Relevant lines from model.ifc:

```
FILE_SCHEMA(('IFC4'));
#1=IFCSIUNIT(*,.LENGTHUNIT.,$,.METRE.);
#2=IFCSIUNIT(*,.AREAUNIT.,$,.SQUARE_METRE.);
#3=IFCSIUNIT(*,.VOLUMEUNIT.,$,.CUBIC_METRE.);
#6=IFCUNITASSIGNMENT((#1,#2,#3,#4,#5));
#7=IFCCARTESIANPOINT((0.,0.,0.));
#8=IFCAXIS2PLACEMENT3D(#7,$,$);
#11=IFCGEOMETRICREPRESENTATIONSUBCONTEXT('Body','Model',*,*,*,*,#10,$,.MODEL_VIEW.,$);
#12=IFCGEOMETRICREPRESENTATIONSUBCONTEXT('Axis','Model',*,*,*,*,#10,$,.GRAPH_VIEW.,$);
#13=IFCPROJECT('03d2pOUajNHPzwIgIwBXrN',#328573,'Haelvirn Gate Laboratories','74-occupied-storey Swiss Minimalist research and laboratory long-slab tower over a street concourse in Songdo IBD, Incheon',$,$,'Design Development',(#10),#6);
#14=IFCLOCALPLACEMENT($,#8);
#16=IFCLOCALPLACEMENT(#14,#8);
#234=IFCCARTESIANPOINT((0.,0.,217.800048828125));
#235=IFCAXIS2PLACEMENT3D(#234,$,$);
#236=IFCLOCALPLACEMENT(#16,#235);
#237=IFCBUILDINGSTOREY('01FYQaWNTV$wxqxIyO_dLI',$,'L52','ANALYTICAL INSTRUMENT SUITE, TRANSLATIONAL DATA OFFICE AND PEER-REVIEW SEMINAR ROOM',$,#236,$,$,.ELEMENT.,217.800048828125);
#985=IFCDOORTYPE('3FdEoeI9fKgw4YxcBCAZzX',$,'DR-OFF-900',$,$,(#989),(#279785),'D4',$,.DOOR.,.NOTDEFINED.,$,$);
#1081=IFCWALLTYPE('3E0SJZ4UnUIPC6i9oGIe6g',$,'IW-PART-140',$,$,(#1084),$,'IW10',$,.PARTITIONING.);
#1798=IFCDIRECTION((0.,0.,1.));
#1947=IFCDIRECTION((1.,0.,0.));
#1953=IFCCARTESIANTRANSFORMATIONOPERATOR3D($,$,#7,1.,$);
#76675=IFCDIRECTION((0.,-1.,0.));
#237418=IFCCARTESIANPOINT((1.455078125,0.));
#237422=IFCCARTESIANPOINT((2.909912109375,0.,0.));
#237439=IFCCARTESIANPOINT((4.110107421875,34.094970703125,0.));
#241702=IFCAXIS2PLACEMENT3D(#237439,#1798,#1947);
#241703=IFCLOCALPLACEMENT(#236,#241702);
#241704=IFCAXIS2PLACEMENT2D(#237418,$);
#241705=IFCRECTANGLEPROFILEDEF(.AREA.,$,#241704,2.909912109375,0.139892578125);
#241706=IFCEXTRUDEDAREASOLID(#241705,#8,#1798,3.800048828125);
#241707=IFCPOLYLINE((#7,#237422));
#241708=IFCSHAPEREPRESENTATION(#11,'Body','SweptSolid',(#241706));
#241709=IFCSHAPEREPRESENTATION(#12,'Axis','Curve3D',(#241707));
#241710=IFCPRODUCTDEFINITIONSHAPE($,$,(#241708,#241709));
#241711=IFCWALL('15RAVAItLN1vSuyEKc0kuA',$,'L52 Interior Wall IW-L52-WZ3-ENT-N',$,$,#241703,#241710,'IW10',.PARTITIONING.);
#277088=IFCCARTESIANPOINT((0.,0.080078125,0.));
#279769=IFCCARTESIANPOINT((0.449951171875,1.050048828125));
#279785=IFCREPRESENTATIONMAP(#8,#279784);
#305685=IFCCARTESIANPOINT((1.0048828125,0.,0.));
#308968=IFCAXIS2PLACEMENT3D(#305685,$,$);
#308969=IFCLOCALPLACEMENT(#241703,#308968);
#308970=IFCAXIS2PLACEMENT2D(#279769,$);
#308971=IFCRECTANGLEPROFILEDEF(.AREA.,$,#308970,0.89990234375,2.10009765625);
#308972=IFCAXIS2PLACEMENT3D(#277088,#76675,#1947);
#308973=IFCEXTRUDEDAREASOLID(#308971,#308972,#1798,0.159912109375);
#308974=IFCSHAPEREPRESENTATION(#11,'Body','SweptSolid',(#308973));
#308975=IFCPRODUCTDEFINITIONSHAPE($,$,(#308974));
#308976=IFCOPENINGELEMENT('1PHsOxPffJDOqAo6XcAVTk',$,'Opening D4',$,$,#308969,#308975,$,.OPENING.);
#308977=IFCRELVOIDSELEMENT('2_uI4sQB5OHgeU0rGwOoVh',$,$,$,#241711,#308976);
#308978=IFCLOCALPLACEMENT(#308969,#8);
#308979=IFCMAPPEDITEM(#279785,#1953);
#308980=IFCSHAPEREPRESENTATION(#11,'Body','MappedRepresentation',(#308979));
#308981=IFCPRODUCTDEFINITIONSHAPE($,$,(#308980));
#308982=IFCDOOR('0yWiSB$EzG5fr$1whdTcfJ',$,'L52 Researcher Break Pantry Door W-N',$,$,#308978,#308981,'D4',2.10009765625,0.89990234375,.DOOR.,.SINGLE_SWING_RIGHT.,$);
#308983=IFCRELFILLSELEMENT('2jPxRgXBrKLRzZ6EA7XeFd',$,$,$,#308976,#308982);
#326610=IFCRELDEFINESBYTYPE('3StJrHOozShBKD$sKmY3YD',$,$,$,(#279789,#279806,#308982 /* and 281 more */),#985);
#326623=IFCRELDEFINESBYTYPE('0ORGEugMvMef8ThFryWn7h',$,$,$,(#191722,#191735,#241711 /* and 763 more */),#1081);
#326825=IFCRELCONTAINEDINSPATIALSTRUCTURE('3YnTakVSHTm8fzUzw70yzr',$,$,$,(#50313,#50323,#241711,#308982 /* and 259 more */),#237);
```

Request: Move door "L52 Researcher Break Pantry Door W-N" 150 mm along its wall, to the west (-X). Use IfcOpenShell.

```python
import ifcopenshell
import ifcopenshell.api.geometry
import ifcopenshell.util.placement
import ifcopenshell.util.unit

model = ifcopenshell.open("model.ifc")
unit_scale = ifcopenshell.util.unit.calculate_unit_scale(model)

door = model.by_guid("0yWiSB$EzG5fr$1whdTcfJ")
opening = door.FillsVoids[0].RelatingOpeningElement
wall = opening.VoidsElements[0].RelatingBuildingElement

wall_matrix = ifcopenshell.util.placement.get_local_placement(wall.ObjectPlacement)
shift = wall_matrix[:3, 0] * -0.15 / unit_scale
before = ifcopenshell.util.placement.get_local_placement(door.ObjectPlacement)[:3, 3].copy()

# The door is placed relative to its opening, so it follows when the opening moves.
matrix = ifcopenshell.util.placement.get_local_placement(opening.ObjectPlacement)
matrix[:3, 3] += shift
ifcopenshell.api.geometry.edit_object_placement(
    model, product=opening, matrix=matrix, is_si=False, should_transform_children=True
)

after = ifcopenshell.util.placement.get_local_placement(door.ObjectPlacement)[:3, 3]
print("door moved by", (after - before).round(3) + 0.0)

model.write("model-out.ifc")
```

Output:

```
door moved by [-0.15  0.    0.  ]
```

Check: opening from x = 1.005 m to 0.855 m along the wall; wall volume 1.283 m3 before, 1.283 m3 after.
